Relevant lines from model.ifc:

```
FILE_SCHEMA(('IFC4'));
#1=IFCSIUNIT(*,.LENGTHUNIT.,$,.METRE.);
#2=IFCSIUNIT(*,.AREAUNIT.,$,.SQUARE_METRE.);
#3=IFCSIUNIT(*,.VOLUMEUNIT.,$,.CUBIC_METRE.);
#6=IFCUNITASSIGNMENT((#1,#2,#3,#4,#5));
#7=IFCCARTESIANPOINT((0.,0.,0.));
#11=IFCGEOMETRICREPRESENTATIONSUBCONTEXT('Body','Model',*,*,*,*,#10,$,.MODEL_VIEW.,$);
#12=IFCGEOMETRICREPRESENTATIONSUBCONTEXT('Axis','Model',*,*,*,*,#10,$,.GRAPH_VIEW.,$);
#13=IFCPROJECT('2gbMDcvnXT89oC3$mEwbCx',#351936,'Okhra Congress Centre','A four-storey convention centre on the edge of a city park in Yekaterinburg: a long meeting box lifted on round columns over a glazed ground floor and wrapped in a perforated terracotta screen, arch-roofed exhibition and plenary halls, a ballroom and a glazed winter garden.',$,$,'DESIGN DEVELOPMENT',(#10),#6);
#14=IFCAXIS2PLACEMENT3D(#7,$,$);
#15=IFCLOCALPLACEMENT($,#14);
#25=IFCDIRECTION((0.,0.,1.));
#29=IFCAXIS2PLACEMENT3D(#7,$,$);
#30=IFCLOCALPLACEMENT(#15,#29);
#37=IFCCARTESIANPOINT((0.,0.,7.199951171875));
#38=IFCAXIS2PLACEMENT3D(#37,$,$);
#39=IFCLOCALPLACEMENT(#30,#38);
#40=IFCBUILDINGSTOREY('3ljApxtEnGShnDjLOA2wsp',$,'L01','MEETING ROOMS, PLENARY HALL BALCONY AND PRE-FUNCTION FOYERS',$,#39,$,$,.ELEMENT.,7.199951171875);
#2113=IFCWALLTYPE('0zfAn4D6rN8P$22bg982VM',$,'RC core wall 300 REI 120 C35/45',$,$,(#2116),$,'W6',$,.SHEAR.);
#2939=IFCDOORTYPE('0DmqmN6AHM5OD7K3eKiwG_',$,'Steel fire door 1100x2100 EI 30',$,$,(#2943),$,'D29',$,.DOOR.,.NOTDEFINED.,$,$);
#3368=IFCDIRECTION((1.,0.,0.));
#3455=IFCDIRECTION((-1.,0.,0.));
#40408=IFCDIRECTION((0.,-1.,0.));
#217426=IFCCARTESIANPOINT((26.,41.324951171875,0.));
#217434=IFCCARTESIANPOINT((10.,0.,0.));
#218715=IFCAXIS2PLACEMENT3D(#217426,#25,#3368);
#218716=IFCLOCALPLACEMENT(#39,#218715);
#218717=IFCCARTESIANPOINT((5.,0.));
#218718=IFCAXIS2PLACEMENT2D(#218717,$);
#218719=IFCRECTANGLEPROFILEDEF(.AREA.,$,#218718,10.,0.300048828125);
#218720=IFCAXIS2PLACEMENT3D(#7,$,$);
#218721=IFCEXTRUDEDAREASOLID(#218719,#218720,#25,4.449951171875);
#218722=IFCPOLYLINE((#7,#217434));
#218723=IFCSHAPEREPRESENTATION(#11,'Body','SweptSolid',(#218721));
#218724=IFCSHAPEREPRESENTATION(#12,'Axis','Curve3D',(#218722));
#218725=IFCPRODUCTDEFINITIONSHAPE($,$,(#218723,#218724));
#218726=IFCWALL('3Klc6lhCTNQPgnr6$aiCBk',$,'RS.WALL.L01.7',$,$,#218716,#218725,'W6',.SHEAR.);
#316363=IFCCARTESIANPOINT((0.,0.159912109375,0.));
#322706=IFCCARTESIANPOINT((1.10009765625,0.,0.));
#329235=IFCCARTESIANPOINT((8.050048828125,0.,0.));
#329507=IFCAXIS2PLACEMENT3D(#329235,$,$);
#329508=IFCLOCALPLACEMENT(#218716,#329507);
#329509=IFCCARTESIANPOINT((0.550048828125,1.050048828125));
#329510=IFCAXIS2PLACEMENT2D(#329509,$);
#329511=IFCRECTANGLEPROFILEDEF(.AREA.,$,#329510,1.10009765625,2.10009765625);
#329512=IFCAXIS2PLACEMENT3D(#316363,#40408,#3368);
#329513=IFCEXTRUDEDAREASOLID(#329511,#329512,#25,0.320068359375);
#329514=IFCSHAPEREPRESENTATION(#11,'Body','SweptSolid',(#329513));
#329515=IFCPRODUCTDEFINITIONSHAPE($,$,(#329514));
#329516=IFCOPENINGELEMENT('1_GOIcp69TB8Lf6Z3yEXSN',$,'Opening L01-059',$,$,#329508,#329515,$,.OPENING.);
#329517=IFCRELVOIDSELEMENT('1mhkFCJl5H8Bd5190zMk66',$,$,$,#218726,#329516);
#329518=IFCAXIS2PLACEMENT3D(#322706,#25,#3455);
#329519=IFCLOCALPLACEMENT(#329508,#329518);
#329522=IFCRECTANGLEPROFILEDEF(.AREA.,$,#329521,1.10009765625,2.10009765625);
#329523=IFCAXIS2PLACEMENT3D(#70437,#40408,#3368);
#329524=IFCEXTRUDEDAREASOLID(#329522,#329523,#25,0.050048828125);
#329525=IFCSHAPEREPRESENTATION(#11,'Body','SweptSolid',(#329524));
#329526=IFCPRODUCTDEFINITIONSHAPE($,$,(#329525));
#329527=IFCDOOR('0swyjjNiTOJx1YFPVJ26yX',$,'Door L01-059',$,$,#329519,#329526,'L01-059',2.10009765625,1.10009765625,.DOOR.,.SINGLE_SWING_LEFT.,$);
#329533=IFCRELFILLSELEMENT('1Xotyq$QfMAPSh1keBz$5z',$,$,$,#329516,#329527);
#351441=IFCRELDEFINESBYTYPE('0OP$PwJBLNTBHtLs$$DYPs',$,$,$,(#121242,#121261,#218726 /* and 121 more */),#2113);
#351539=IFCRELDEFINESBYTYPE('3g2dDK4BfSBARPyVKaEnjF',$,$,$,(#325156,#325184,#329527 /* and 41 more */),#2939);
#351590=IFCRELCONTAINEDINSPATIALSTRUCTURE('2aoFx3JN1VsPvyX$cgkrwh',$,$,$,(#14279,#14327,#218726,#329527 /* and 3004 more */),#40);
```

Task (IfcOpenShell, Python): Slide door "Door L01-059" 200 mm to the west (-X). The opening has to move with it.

```python
import ifcopenshell
import ifcopenshell.api.geometry
import ifcopenshell.util.placement
import ifcopenshell.util.unit

model = ifcopenshell.open("model.ifc")
unit_scale = ifcopenshell.util.unit.calculate_unit_scale(model)

door = model.by_id(329527)
opening = door.FillsVoids[0].RelatingOpeningElement
wall = opening.VoidsElements[0].RelatingBuildingElement

wall_matrix = ifcopenshell.util.placement.get_local_placement(wall.ObjectPlacement)
shift = wall_matrix[:3, 0] * -0.2 / unit_scale
before = ifcopenshell.util.placement.get_local_placement(door.ObjectPlacement)[:3, 3].copy()

# The door is placed relative to its opening, so it follows when the opening moves.
matrix = ifcopenshell.util.placement.get_local_placement(opening.ObjectPlacement)
matrix[:3, 3] += shift
ifcopenshell.api.geometry.edit_object_placement(
    model, product=opening, matrix=matrix, is_si=False, should_transform_children=True
)

after = ifcopenshell.util.placement.get_local_placement(door.ObjectPlacement)[:3, 3]
print("door moved by", (after - before).round(3) + 0.0)

model.write("model_edited.ifc")
```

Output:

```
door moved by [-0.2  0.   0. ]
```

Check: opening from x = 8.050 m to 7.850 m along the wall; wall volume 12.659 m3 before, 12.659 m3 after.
